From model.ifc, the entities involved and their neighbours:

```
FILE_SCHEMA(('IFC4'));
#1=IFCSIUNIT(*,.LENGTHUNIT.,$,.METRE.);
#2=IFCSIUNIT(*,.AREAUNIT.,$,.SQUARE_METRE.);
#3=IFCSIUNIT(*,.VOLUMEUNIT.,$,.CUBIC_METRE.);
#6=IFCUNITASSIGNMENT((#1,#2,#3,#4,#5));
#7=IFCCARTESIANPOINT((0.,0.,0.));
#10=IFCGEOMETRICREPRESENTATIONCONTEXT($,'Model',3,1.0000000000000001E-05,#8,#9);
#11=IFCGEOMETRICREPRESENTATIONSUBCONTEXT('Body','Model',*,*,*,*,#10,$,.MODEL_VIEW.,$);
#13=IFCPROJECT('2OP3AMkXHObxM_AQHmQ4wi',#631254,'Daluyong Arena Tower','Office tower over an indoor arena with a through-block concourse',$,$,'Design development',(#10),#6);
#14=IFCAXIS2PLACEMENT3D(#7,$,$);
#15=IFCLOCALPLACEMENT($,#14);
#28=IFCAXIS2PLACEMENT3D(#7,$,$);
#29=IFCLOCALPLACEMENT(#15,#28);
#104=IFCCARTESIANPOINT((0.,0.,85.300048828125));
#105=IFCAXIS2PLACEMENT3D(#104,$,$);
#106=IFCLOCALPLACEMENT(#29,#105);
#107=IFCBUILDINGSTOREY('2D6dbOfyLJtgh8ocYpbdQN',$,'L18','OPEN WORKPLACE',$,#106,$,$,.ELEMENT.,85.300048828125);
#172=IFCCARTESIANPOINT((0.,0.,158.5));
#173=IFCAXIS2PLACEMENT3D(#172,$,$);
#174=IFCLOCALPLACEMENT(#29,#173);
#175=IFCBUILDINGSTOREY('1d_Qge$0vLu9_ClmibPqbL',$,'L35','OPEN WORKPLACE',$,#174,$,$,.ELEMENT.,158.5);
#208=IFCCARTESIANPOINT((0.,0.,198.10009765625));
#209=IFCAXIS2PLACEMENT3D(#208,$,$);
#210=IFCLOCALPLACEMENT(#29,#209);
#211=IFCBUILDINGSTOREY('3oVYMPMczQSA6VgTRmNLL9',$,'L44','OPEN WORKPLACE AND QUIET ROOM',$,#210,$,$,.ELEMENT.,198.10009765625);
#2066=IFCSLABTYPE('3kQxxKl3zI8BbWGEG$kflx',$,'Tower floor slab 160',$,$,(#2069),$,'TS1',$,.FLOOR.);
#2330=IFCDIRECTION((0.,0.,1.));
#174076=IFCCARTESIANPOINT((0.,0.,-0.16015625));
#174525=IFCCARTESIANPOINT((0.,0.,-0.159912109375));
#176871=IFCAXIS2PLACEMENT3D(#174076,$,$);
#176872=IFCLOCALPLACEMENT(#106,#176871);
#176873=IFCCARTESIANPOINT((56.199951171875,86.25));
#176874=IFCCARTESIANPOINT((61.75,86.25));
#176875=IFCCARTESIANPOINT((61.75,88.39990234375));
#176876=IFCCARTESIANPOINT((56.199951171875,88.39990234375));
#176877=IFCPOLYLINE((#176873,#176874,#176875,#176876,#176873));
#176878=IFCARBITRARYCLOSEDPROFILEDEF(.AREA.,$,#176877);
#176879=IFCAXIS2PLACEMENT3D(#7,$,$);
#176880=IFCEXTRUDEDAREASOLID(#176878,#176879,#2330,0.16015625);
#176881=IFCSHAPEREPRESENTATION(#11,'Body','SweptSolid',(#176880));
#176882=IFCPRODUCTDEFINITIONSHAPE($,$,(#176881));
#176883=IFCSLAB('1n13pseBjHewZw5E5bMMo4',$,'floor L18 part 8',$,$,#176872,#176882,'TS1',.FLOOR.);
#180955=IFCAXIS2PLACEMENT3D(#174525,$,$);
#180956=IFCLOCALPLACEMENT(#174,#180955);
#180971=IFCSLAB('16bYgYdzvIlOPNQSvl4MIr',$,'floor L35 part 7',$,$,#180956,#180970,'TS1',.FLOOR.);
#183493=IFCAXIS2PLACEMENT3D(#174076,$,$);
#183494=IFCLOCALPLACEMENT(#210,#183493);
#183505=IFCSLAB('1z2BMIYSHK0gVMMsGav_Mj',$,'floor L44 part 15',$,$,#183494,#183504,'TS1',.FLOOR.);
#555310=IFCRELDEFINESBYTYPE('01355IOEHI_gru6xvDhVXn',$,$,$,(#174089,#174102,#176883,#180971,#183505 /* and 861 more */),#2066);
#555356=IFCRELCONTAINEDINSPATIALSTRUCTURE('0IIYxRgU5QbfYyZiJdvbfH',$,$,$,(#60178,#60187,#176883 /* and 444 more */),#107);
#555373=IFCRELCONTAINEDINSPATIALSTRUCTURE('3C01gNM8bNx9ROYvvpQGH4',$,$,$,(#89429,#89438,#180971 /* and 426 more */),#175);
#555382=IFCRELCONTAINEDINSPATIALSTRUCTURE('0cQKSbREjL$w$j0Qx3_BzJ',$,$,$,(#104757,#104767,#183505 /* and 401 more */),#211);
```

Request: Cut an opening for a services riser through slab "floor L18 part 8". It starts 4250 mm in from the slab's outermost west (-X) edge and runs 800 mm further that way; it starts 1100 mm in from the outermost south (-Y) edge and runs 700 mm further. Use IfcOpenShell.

```python
import numpy as np
import ifcopenshell
import ifcopenshell.api.feature
import ifcopenshell.api.geometry
import ifcopenshell.api.root
import ifcopenshell.geom
import ifcopenshell.util.placement
import ifcopenshell.util.representation
import ifcopenshell.util.shape
import ifcopenshell.util.unit

model = ifcopenshell.open("model.ifc")
unit_scale = ifcopenshell.util.unit.calculate_unit_scale(model)
settings = ifcopenshell.geom.settings()


def volume(element):
    """Net volume in cubic metres, openings subtracted."""
    shape = ifcopenshell.geom.create_shape(settings, element)
    return ifcopenshell.util.shape.get_volume(shape.geometry)


slab = model.by_id(176883)
before = volume(slab)

# Extent in the slab's own axes, in metres. The edges named are its -X and -Y sides.
slab_shape = ifcopenshell.geom.create_shape(settings, slab)
vertices = ifcopenshell.util.shape.get_vertices(slab_shape.geometry)
x_min, y_min, bottom = vertices.min(axis=0)
top = vertices[:, 2].max()

opening = ifcopenshell.api.root.create_entity(model, ifc_class="IfcOpeningElement", name="Services riser opening", predefined_type="OPENING")
context = ifcopenshell.util.representation.get_context(model, "Model", "Body", "MODEL_VIEW")
width, depth = 0.8, 0.7
outline = [(0.0, 0.0), (width, 0.0), (width, depth), (0.0, depth), (0.0, 0.0)]
# Overshoot both faces by 50 mm so the cut is clean.
shape = ifcopenshell.api.geometry.add_slab_representation(
    model, context=context, depth=top - bottom + 0.1, polyline=outline
)
ifcopenshell.api.geometry.assign_representation(model, product=opening, representation=shape)

matrix = ifcopenshell.util.placement.get_local_placement(slab.ObjectPlacement)
matrix[:, 3] = matrix @ np.append(np.array([x_min + 4.25, y_min + 1.1, bottom - 0.05]) / unit_scale, 1.0)
ifcopenshell.api.geometry.edit_object_placement(model, product=opening, matrix=matrix, is_si=False)
ifcopenshell.api.feature.add_feature(model, feature=opening, element=slab)

after = volume(slab)

print(f"slab volume {before:.3f} -> {after:.3f} m3")

model.write("model_edited.ifc")
```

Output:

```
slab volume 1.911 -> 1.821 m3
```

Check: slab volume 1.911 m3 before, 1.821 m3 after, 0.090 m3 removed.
